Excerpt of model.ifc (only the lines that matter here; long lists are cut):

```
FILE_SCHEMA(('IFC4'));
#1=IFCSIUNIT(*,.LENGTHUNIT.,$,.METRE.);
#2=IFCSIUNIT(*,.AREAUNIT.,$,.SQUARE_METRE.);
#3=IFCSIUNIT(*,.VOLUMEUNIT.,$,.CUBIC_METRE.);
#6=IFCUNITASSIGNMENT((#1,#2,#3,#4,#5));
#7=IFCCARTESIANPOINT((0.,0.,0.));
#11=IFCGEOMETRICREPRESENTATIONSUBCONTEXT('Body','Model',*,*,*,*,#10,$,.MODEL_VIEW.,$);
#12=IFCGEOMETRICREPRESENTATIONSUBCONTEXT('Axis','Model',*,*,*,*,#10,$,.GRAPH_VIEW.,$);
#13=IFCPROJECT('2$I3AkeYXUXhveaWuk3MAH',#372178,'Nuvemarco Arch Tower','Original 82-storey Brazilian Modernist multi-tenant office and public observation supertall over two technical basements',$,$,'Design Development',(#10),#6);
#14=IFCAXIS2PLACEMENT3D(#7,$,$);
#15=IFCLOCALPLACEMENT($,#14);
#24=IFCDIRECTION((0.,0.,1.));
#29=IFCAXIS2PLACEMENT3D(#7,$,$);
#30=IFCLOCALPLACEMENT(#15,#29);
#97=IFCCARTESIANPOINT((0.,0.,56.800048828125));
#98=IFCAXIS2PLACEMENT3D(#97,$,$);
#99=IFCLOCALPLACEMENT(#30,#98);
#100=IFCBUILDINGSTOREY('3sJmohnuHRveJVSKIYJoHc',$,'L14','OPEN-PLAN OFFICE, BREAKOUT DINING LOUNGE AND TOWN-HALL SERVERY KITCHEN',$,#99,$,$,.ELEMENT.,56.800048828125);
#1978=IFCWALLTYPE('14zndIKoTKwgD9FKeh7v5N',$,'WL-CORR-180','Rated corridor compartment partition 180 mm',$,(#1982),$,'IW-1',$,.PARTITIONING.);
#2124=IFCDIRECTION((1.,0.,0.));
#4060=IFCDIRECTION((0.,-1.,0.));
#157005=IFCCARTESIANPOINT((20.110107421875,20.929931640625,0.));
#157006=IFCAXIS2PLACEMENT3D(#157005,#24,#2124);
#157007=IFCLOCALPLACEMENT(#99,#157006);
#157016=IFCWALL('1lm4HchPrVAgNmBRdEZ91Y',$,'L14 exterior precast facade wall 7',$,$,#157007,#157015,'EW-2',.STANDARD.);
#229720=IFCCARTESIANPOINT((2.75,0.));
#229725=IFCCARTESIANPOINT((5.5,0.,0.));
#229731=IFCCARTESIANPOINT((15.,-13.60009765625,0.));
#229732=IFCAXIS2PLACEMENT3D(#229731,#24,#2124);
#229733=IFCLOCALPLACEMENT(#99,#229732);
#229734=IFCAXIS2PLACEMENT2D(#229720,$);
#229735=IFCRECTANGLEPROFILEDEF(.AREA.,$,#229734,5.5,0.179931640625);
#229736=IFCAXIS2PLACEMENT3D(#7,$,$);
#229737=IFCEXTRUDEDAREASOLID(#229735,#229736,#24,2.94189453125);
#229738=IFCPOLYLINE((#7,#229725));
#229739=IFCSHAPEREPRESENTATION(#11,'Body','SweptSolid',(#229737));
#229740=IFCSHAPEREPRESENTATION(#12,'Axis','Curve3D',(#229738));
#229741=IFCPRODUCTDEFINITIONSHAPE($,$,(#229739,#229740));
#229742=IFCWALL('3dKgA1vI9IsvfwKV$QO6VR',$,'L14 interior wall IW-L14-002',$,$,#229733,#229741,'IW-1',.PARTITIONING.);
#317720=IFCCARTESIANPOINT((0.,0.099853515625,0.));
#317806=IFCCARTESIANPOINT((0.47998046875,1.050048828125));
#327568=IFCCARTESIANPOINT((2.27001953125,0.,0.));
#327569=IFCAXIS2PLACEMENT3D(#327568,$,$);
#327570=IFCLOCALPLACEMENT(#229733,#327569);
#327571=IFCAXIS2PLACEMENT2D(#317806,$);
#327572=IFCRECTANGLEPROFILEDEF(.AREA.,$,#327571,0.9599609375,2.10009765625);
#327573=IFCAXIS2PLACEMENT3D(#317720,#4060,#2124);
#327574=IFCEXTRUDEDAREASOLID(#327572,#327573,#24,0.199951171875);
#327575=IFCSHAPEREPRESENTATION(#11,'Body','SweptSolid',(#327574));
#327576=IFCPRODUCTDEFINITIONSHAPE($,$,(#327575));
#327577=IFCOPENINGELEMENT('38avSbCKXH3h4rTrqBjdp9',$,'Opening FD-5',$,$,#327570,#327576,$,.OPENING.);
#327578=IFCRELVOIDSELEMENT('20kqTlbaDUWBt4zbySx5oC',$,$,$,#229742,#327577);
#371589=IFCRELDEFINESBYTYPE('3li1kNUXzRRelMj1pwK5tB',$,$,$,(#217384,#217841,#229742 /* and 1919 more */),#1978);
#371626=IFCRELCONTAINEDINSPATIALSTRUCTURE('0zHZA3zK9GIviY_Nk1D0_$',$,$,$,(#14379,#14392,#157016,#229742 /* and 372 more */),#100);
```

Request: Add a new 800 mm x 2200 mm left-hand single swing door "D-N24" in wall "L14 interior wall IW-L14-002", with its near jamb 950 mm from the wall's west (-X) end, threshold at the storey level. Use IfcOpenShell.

```python
import numpy as np
import ifcopenshell
import ifcopenshell.api.feature
import ifcopenshell.api.geometry
import ifcopenshell.api.root
import ifcopenshell.api.spatial
import ifcopenshell.geom
import ifcopenshell.util.element
import ifcopenshell.util.placement
import ifcopenshell.util.representation
import ifcopenshell.util.shape
import ifcopenshell.util.unit

model = ifcopenshell.open("model.ifc")
unit_scale = ifcopenshell.util.unit.calculate_unit_scale(model)
settings = ifcopenshell.geom.settings()


def volume(element):
    """Net volume in cubic metres, openings subtracted."""
    shape = ifcopenshell.geom.create_shape(settings, element)
    return ifcopenshell.util.shape.get_volume(shape.geometry)


wall = model.by_guid("3dKgA1vI9IsvfwKV$QO6VR")
storey = ifcopenshell.util.element.get_container(wall, ifc_class="IfcBuildingStorey")
context = ifcopenshell.util.representation.get_context(model, "Model", "Body", "MODEL_VIEW")
before = volume(wall)

width, height, from_end, sill = 0.8, 2.2, 0.95, 0.0  # metres

# The wall runs along its own X axis, and the end named is its -X end.
wall_shape = ifcopenshell.geom.create_shape(settings, wall)
x, y, z = ifcopenshell.util.shape.get_vertices(wall_shape.geometry).T
start = x.min() + from_end
face, thickness = float(y.min()), float(y.max() - y.min())
wall_matrix = ifcopenshell.util.placement.get_local_placement(wall.ObjectPlacement)
level = ifcopenshell.util.placement.get_local_placement(storey.ObjectPlacement)[2, 3]


def in_wall(x, y):
    """Placement at x, y metres in the wall's axes, at sill height."""
    matrix = wall_matrix.copy()
    matrix[:, 3] = wall_matrix @ np.array([x / unit_scale, y / unit_scale, 0.0, 1.0])
    matrix[2, 3] = level + sill / unit_scale
    return matrix


# Opening: a box that overshoots both wall faces by 50 mm.
opening = ifcopenshell.api.root.create_entity(model, ifc_class="IfcOpeningElement", predefined_type="OPENING")
box = ifcopenshell.api.geometry.add_wall_representation(
    model, context=context, length=width, height=height, thickness=thickness + 0.1
)
ifcopenshell.api.geometry.assign_representation(model, product=opening, representation=box)
ifcopenshell.api.geometry.edit_object_placement(model, product=opening, matrix=in_wall(start, face - 0.05), is_si=False)
ifcopenshell.api.feature.add_feature(model, feature=opening, element=wall)

door = ifcopenshell.api.root.create_entity(model, ifc_class="IfcDoor", name="D-N24", predefined_type="DOOR")
door.OverallWidth, door.OverallHeight = width / unit_scale, height / unit_scale
door.OperationType = "SINGLE_SWING_LEFT"
body = ifcopenshell.api.geometry.add_door_representation(
    model,
    context=context,
    overall_width=door.OverallWidth,
    overall_height=door.OverallHeight,
    operation_type="SINGLE_SWING_LEFT",
    lining_properties={"LiningDepth": thickness / unit_scale, "ThresholdDepth": thickness / unit_scale},
)
ifcopenshell.api.geometry.assign_representation(model, product=door, representation=body)
ifcopenshell.api.spatial.assign_container(model, products=[door], relating_structure=storey)
ifcopenshell.api.feature.add_filling(model, opening=opening, element=door)

# The lining spans the wall, so the door starts at the wall face.
ifcopenshell.api.geometry.edit_object_placement(model, product=door, matrix=in_wall(start, face), is_si=False)

after = volume(wall)

print(f"wall volume {before:.3f} -> {after:.3f} m3")

model.write("model_rev.ifc")
```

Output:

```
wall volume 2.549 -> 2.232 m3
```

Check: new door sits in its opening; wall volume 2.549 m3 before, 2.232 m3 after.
